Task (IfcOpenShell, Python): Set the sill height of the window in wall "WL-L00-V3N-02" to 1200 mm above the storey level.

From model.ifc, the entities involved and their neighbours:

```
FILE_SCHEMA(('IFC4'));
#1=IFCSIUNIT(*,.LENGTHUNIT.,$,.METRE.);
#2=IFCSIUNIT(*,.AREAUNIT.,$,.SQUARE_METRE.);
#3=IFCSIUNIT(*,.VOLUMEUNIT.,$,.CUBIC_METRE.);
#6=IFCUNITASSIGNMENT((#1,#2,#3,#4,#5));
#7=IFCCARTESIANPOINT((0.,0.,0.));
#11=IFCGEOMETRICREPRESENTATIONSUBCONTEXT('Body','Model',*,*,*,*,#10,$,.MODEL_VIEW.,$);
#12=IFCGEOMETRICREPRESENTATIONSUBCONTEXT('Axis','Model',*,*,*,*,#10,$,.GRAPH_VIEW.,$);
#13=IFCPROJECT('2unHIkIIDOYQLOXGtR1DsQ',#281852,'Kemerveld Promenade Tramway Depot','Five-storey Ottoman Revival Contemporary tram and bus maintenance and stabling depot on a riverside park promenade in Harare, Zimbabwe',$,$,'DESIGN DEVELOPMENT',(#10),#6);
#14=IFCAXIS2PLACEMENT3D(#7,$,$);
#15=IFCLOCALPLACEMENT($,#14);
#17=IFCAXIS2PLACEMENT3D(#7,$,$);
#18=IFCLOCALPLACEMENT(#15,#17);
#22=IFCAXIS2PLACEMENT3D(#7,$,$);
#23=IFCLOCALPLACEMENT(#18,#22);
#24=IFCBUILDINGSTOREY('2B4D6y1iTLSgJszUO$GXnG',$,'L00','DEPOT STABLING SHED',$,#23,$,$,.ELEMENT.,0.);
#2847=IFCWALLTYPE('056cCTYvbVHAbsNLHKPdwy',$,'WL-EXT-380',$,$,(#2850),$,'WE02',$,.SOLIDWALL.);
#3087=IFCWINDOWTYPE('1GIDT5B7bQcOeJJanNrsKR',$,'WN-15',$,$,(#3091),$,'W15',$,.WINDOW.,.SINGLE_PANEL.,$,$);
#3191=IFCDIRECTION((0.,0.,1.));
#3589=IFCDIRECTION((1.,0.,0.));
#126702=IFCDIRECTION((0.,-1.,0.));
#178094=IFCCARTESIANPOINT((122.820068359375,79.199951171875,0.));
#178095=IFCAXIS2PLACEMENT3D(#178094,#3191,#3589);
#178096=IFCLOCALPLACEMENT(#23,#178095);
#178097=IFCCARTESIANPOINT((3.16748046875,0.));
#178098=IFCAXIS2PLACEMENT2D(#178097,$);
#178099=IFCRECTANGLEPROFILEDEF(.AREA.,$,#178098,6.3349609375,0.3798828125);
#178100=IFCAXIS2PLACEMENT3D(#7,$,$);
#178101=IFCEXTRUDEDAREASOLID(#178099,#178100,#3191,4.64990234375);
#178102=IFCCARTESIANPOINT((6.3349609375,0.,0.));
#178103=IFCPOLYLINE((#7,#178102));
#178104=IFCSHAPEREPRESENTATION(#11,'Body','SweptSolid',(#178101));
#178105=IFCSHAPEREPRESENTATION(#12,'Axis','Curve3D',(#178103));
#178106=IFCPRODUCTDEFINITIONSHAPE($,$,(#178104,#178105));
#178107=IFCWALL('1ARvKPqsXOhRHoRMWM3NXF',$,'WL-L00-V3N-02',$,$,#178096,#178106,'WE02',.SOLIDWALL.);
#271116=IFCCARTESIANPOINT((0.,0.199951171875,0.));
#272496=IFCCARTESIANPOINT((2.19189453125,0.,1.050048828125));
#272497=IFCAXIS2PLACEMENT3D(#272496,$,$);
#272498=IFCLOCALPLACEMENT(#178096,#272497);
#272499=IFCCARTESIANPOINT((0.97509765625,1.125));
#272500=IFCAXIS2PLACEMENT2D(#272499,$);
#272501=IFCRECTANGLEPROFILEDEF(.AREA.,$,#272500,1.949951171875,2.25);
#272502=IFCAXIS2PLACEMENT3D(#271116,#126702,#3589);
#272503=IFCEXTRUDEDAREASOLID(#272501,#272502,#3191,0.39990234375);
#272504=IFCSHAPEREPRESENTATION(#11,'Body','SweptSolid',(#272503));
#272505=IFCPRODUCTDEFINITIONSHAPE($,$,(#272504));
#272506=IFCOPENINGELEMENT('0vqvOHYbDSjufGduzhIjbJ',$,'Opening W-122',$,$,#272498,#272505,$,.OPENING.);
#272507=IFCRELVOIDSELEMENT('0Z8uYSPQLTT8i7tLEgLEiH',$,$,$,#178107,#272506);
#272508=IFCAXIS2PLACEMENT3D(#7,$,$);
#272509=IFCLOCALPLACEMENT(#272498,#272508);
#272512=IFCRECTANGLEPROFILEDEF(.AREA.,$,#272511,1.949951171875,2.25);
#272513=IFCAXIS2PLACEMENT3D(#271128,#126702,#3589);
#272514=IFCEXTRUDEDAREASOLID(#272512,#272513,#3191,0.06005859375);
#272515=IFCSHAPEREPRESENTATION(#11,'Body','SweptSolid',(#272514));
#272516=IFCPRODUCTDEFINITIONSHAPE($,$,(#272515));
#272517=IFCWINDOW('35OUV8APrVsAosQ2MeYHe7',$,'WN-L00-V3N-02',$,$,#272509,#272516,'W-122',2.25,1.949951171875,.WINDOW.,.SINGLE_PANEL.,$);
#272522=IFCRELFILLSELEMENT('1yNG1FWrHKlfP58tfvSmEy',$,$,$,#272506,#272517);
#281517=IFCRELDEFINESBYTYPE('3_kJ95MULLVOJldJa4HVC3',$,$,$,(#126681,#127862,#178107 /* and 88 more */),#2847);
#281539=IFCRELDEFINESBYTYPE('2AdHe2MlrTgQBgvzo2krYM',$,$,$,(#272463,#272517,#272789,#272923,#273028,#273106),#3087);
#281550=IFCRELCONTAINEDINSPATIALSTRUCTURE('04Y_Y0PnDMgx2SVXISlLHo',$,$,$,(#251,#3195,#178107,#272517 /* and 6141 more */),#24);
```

```python
import numpy as np
import ifcopenshell
import ifcopenshell.api.geometry
import ifcopenshell.geom
import ifcopenshell.util.element
import ifcopenshell.util.placement
import ifcopenshell.util.shape
import ifcopenshell.util.unit

model = ifcopenshell.open("model.ifc")
unit_scale = ifcopenshell.util.unit.calculate_unit_scale(model)

window = model.by_id(272517)
opening = window.FillsVoids[0].RelatingOpeningElement
storey = ifcopenshell.util.element.get_container(window, ifc_class="IfcBuildingStorey")
level = ifcopenshell.util.placement.get_local_placement(storey.ObjectPlacement)[2, 3]

# The opening's origin need not be at the sill, so measure its lowest point.
shape = ifcopenshell.geom.create_shape(ifcopenshell.geom.settings(), opening)
bottom = ifcopenshell.util.shape.get_shape_bottom_elevation(shape, shape.geometry) / unit_scale
dz = level + 1.2 - bottom

shift = np.array([0.0, 0.0, dz])
# The window is placed relative to its opening, so it follows when the opening moves.
matrix = ifcopenshell.util.placement.get_local_placement(opening.ObjectPlacement)
matrix[:3, 3] += shift
ifcopenshell.api.geometry.edit_object_placement(
    model, product=opening, matrix=matrix, is_si=False, should_transform_children=True
)

print(f"moved by {dz * unit_scale:+.3f} m")

model.write("model_updated.ifc")
```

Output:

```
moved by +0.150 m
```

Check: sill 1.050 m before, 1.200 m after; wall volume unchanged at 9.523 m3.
